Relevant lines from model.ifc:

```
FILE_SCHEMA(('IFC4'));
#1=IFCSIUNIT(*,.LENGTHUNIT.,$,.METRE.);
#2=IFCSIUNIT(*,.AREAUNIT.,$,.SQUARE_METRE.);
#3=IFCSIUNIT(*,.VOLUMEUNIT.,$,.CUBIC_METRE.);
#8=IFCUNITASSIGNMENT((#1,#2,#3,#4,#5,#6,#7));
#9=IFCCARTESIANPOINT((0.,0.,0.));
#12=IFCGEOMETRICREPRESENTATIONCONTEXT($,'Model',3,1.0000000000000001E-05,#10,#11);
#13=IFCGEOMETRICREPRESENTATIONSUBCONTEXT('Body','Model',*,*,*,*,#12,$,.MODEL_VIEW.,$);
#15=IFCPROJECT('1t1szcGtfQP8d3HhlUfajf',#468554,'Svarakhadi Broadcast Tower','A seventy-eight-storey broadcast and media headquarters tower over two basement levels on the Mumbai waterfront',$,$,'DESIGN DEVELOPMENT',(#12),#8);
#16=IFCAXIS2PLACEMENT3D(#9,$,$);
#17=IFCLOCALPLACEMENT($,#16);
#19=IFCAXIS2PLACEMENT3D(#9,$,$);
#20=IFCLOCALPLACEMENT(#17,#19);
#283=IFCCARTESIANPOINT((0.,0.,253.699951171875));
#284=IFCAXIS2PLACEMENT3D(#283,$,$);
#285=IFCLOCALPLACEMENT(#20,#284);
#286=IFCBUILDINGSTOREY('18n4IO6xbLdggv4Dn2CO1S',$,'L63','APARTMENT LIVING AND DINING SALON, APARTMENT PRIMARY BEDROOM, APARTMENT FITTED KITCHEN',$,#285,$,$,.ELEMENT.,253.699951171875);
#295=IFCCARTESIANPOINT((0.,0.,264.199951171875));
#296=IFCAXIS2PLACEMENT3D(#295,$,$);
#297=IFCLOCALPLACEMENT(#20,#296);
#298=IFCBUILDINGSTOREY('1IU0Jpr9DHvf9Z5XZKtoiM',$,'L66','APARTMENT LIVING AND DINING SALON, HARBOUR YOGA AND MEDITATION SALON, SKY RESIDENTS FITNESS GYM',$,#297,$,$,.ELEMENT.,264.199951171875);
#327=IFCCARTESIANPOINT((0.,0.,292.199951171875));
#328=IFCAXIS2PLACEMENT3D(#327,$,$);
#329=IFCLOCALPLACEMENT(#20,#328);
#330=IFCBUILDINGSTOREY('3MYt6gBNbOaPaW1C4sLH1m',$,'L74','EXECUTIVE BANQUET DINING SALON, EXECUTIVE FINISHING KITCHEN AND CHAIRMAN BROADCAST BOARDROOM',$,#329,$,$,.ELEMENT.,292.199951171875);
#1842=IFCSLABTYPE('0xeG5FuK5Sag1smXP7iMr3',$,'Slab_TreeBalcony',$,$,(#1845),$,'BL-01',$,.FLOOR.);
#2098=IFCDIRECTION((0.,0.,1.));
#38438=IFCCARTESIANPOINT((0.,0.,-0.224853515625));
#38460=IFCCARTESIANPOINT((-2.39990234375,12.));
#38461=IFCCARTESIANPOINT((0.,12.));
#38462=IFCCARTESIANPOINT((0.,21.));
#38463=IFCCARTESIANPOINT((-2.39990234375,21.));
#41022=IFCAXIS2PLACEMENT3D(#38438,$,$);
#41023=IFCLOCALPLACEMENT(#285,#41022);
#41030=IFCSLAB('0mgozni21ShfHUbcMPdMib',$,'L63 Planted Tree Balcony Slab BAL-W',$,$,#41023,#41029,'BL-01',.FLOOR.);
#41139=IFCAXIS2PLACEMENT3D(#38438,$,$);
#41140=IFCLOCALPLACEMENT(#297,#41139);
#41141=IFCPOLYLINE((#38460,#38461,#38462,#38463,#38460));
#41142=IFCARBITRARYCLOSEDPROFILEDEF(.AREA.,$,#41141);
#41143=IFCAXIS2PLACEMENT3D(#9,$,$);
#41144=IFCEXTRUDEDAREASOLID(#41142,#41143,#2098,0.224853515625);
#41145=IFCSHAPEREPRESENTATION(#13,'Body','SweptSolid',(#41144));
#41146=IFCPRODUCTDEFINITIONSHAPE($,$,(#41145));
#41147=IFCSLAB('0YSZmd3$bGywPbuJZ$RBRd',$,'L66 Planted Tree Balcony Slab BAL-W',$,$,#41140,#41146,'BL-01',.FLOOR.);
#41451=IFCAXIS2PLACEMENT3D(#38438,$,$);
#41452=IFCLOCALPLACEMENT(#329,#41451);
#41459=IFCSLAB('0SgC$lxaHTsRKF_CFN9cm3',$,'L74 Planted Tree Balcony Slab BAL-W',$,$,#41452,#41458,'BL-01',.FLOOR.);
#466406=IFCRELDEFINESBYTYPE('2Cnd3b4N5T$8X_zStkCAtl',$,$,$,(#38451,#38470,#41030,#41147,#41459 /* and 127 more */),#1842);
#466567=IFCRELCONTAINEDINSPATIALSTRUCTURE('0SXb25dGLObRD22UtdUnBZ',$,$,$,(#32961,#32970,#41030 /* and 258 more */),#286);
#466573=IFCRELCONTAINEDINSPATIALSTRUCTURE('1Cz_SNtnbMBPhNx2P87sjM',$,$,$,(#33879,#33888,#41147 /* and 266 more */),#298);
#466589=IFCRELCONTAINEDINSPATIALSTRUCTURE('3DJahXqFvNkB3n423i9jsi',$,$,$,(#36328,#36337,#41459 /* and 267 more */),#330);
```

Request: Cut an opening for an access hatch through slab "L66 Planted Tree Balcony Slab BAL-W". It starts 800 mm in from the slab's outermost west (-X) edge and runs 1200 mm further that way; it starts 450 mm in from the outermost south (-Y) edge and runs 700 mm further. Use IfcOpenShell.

```python
import numpy as np
import ifcopenshell
import ifcopenshell.api.feature
import ifcopenshell.api.geometry
import ifcopenshell.api.root
import ifcopenshell.geom
import ifcopenshell.util.placement
import ifcopenshell.util.representation
import ifcopenshell.util.shape
import ifcopenshell.util.unit

model = ifcopenshell.open("model.ifc")
unit_scale = ifcopenshell.util.unit.calculate_unit_scale(model)
settings = ifcopenshell.geom.settings()


def volume(element):
    """Net volume in cubic metres, openings subtracted."""
    shape = ifcopenshell.geom.create_shape(settings, element)
    return ifcopenshell.util.shape.get_volume(shape.geometry)


slab = model.by_guid("0YSZmd3$bGywPbuJZ$RBRd")
before = volume(slab)

# Extent in the slab's own axes, in metres. The edges named are its -X and -Y sides.
slab_shape = ifcopenshell.geom.create_shape(settings, slab)
vertices = ifcopenshell.util.shape.get_vertices(slab_shape.geometry)
x_min, y_min, bottom = vertices.min(axis=0)
top = vertices[:, 2].max()

opening = ifcopenshell.api.root.create_entity(model, ifc_class="IfcOpeningElement", name="Access hatch opening", predefined_type="OPENING")
context = ifcopenshell.util.representation.get_context(model, "Model", "Body", "MODEL_VIEW")
width, depth = 1.2, 0.7
outline = [(0.0, 0.0), (width, 0.0), (width, depth), (0.0, depth), (0.0, 0.0)]
# Overshoot both faces by 50 mm so the cut is clean.
shape = ifcopenshell.api.geometry.add_slab_representation(
    model, context=context, depth=top - bottom + 0.1, polyline=outline
)
ifcopenshell.api.geometry.assign_representation(model, product=opening, representation=shape)

matrix = ifcopenshell.util.placement.get_local_placement(slab.ObjectPlacement)
matrix[:, 3] = matrix @ np.append(np.array([x_min + 0.8, y_min + 0.45, bottom - 0.05]) / unit_scale, 1.0)
ifcopenshell.api.geometry.edit_object_placement(model, product=opening, matrix=matrix, is_si=False)
ifcopenshell.api.feature.add_feature(model, feature=opening, element=slab)

after = volume(slab)

print(f"slab volume {before:.3f} -> {after:.3f} m3")

model.write("model_rev.ifc")
```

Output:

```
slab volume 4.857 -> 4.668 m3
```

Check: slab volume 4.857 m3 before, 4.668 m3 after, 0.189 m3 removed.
